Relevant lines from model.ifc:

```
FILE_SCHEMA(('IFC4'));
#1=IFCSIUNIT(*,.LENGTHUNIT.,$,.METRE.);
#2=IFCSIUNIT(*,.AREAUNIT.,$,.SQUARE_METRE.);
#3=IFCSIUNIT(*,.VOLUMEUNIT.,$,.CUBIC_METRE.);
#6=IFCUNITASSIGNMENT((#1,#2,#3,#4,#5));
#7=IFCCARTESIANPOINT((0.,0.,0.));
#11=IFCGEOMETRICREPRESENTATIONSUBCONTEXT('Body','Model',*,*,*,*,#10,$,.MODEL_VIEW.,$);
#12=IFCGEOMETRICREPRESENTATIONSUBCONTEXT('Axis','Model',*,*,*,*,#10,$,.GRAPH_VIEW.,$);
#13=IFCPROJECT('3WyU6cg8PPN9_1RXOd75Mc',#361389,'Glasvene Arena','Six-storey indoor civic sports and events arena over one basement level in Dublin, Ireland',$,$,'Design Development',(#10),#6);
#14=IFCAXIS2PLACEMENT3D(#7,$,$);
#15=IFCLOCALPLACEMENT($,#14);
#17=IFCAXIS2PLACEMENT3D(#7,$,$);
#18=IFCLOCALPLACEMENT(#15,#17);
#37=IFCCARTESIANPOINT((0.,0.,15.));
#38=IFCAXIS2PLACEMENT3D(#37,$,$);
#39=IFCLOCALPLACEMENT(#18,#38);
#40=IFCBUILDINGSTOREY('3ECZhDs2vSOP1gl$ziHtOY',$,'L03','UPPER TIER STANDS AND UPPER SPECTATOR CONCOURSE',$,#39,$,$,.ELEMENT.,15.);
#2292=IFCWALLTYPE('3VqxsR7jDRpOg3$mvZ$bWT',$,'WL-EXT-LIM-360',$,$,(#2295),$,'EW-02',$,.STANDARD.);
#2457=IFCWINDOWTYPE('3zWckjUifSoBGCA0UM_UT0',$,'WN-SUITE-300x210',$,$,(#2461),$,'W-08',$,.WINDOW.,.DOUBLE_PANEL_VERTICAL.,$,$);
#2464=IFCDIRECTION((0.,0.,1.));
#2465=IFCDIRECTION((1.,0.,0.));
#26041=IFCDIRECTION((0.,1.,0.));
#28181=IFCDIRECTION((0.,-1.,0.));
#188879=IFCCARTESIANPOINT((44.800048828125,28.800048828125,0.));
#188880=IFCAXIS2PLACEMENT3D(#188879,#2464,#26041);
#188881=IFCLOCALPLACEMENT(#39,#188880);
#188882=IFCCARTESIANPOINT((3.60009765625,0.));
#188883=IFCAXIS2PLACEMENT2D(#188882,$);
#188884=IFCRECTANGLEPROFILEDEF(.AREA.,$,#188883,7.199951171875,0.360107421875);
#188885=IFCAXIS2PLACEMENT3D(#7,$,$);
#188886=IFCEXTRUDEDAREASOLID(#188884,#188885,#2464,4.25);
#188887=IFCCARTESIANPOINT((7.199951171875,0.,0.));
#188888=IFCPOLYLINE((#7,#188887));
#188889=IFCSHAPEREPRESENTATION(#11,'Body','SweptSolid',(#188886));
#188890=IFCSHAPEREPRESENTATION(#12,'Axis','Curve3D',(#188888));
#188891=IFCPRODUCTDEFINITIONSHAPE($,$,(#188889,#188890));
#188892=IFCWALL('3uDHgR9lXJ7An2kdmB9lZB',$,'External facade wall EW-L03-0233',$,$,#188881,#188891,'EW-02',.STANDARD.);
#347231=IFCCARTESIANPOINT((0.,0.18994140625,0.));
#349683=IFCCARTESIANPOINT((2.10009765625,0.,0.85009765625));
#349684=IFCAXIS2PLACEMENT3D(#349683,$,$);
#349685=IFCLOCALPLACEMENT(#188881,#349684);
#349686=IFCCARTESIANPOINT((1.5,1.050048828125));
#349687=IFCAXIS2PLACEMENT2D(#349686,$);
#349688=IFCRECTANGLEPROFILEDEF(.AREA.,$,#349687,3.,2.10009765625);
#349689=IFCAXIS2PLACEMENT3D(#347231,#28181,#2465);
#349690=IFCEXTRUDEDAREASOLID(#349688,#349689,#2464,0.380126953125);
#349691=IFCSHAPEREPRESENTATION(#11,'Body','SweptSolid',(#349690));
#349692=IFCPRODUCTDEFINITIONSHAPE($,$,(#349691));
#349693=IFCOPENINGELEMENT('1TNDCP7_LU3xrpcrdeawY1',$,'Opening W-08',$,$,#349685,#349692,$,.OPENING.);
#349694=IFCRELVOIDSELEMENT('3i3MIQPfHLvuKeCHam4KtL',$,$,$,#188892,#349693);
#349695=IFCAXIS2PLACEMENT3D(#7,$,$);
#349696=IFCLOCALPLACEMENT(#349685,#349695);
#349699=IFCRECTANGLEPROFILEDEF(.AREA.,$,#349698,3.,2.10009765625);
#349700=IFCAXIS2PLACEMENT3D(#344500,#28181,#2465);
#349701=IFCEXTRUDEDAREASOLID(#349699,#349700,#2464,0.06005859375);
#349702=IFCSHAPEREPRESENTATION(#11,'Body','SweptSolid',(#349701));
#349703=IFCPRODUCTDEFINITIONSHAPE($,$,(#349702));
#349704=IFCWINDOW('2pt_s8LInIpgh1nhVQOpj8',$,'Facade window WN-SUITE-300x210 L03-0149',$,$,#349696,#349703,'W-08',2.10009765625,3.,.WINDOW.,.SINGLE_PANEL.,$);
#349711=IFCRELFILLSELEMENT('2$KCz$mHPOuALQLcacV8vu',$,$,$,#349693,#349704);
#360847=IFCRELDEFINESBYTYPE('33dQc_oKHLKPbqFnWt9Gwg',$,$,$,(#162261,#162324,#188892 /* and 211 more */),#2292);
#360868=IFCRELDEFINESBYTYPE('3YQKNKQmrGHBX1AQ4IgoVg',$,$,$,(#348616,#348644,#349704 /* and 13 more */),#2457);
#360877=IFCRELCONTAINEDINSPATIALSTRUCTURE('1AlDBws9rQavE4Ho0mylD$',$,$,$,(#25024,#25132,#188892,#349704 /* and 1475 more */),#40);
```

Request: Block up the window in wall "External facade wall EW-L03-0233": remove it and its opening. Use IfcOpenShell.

```python
import ifcopenshell
import ifcopenshell.api.feature
import ifcopenshell.api.root
import ifcopenshell.geom
import ifcopenshell.util.shape

model = ifcopenshell.open("model.ifc")
settings = ifcopenshell.geom.settings()


def volume(element):
    """Net volume in cubic metres, openings subtracted."""
    shape = ifcopenshell.geom.create_shape(settings, element)
    return ifcopenshell.util.shape.get_volume(shape.geometry)


window = model.by_id(349704)
opening = window.FillsVoids[0].RelatingOpeningElement
wall = opening.VoidsElements[0].RelatingBuildingElement
before = volume(wall)

ifcopenshell.api.root.remove_product(model, product=window)
ifcopenshell.api.feature.remove_feature(model, feature=opening)

after = volume(wall)

print(f"wall volume {before:.3f} -> {after:.3f} m3")

model.write("model_rev.ifc")
```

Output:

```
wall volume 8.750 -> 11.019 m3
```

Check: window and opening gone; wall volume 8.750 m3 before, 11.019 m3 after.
